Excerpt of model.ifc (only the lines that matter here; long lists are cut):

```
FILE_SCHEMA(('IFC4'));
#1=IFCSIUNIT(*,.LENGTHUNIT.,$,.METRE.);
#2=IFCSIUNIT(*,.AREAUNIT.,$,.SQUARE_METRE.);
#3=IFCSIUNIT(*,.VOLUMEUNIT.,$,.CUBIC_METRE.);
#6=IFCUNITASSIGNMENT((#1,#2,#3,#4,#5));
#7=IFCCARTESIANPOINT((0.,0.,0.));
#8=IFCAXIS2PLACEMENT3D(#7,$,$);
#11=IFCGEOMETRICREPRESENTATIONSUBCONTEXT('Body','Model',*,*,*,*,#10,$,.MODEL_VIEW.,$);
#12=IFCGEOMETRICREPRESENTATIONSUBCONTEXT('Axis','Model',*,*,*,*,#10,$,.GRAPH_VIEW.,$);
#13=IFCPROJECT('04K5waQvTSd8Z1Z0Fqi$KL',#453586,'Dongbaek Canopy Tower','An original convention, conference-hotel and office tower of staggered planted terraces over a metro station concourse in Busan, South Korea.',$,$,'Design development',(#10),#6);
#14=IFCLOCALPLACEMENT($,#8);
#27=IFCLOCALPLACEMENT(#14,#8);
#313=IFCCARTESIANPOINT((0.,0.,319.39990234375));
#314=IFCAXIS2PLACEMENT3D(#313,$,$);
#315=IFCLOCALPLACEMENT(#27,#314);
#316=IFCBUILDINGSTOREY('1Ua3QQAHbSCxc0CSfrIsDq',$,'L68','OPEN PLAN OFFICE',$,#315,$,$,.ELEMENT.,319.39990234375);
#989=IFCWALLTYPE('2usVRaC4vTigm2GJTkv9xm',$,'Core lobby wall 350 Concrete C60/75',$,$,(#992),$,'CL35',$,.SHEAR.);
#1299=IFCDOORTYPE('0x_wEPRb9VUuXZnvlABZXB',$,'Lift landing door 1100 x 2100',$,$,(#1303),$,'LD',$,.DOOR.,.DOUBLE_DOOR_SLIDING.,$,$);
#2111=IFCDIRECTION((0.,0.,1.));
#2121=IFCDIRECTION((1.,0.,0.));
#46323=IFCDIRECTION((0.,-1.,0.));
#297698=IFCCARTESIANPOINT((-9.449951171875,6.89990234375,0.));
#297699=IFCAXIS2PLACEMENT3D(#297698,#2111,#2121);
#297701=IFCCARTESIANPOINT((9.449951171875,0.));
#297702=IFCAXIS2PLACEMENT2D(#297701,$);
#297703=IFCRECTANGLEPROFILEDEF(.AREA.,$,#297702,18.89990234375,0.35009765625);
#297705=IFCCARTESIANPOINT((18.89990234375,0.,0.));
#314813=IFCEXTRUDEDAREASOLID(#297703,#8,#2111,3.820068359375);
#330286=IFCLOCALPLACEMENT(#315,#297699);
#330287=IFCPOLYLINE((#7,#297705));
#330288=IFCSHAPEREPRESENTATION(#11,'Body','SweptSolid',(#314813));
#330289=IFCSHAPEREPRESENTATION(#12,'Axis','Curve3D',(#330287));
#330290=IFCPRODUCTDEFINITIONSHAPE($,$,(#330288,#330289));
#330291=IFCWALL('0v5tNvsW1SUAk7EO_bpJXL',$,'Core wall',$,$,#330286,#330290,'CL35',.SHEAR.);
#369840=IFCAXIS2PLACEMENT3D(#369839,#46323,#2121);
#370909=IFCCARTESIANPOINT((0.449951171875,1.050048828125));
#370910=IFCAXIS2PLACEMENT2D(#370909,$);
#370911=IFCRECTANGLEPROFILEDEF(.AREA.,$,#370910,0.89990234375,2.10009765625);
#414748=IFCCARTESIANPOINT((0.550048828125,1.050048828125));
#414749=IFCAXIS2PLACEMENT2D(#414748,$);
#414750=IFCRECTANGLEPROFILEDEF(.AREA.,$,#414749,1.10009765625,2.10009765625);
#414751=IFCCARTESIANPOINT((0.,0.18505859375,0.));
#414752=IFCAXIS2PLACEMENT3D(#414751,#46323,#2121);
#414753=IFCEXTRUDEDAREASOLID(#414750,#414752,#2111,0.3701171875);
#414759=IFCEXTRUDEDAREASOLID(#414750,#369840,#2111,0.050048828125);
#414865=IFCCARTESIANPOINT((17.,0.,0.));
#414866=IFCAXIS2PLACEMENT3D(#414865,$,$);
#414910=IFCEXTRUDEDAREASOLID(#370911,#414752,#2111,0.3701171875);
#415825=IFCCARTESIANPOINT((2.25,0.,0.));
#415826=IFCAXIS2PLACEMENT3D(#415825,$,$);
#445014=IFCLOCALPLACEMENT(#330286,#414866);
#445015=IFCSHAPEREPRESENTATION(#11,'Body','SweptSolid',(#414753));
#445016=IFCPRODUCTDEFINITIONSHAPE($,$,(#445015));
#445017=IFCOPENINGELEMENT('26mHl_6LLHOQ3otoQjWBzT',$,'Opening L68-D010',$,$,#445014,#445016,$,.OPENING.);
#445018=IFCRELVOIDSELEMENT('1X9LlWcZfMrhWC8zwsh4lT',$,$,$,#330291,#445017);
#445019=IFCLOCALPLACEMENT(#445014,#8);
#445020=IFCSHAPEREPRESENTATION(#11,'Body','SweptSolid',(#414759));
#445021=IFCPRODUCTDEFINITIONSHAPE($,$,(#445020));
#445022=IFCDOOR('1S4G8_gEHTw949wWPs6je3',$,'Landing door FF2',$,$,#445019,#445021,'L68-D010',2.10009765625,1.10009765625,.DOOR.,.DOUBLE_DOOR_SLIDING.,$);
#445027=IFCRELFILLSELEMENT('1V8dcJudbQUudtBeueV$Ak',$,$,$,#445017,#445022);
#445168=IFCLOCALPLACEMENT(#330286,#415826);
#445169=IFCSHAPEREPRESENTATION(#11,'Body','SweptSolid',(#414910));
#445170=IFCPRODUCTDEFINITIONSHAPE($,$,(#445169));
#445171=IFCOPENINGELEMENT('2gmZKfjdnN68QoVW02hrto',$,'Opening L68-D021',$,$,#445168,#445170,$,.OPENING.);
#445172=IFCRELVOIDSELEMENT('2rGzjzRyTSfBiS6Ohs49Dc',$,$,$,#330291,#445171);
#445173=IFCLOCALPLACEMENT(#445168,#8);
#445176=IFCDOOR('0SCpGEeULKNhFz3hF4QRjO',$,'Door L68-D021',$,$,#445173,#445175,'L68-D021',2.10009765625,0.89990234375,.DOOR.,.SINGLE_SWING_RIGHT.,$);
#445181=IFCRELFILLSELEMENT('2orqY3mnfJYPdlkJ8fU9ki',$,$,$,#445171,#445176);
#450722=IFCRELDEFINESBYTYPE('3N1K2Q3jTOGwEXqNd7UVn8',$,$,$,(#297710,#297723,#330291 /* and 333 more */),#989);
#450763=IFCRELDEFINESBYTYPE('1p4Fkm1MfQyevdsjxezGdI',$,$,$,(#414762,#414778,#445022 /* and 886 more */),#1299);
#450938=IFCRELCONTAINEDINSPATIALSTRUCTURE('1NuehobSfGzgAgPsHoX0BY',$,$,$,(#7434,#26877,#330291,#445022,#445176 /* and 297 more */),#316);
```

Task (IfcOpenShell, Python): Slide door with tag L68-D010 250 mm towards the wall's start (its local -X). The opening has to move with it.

```python
import ifcopenshell
import ifcopenshell.api.geometry
import ifcopenshell.util.placement

model = ifcopenshell.open("model.ifc")

door = model.by_guid("1S4G8_gEHTw949wWPs6je3")
opening = door.FillsVoids[0].RelatingOpeningElement
wall = opening.VoidsElements[0].RelatingBuildingElement

wall_matrix = ifcopenshell.util.placement.get_local_placement(wall.ObjectPlacement)
shift = wall_matrix[:3, 0] * -0.25
before = ifcopenshell.util.placement.get_local_placement(door.ObjectPlacement)[:3, 3].copy()

# The door is placed relative to its opening, so it follows when the opening moves.
matrix = ifcopenshell.util.placement.get_local_placement(opening.ObjectPlacement)
matrix[:3, 3] += shift
ifcopenshell.api.geometry.edit_object_placement(
    model, product=opening, matrix=matrix, is_si=False, should_transform_children=True
)

after = ifcopenshell.util.placement.get_local_placement(door.ObjectPlacement)[:3, 3]
print("door moved by", (after - before).round(3) + 0.0)

model.write("model_edited.ifc")
```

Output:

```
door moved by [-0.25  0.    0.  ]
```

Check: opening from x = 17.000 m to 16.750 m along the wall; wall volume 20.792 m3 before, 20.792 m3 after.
